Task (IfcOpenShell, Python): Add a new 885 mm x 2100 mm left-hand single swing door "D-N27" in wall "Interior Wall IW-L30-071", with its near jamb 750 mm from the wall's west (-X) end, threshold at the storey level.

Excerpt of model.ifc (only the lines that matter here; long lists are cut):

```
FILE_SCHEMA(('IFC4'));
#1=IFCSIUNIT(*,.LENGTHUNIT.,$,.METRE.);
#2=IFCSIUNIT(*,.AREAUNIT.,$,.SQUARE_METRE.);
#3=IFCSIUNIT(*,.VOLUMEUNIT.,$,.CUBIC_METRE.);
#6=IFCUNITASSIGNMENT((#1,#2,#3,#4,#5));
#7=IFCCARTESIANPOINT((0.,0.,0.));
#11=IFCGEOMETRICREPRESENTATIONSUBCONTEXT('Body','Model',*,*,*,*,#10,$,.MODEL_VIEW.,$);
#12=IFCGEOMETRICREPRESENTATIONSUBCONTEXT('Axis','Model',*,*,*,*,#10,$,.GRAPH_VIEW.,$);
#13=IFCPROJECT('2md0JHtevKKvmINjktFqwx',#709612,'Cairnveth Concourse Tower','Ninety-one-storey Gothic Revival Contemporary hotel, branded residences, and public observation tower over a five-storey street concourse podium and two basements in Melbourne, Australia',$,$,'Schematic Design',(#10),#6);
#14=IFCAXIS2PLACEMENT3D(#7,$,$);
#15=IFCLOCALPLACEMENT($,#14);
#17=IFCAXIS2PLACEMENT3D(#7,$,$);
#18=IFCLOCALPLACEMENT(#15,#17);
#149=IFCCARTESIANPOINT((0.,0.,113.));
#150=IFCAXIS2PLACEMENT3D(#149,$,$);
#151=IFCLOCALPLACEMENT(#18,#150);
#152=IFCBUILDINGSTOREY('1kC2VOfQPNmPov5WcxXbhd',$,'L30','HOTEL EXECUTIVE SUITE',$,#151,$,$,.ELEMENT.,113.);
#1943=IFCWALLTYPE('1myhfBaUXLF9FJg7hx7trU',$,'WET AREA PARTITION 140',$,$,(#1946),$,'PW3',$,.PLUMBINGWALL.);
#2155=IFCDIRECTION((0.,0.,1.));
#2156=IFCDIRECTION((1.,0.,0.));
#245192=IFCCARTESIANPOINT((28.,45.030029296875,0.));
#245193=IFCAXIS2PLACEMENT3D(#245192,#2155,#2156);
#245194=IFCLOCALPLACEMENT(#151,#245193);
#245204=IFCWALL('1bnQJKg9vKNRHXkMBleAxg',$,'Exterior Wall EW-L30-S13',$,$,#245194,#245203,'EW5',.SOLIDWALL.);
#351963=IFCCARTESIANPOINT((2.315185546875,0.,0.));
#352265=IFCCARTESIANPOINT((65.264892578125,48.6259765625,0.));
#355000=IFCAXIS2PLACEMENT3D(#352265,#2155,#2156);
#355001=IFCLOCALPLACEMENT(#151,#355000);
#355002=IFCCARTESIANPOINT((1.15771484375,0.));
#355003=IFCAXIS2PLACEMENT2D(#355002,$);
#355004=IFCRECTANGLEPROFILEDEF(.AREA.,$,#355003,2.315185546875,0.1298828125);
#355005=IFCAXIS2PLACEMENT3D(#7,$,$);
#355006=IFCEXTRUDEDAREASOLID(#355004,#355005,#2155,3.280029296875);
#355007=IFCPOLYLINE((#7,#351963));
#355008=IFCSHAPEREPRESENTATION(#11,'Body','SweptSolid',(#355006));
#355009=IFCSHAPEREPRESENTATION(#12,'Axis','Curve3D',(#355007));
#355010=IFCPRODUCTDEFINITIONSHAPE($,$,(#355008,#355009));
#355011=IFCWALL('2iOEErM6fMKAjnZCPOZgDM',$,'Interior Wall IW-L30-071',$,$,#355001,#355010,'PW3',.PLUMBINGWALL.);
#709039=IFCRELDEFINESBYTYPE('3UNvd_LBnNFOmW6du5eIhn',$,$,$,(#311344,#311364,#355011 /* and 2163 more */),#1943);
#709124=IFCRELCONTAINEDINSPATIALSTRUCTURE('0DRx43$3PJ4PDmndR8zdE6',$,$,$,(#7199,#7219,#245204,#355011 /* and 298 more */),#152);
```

```python
import numpy as np
import ifcopenshell
import ifcopenshell.api.feature
import ifcopenshell.api.geometry
import ifcopenshell.api.root
import ifcopenshell.api.spatial
import ifcopenshell.geom
import ifcopenshell.util.element
import ifcopenshell.util.placement
import ifcopenshell.util.representation
import ifcopenshell.util.shape
import ifcopenshell.util.unit

model = ifcopenshell.open("model.ifc")
unit_scale = ifcopenshell.util.unit.calculate_unit_scale(model)
settings = ifcopenshell.geom.settings()


def volume(element):
    """Net volume in cubic metres, openings subtracted."""
    shape = ifcopenshell.geom.create_shape(settings, element)
    return ifcopenshell.util.shape.get_volume(shape.geometry)


wall = model.by_guid("2iOEErM6fMKAjnZCPOZgDM")
storey = ifcopenshell.util.element.get_container(wall, ifc_class="IfcBuildingStorey")
context = ifcopenshell.util.representation.get_context(model, "Model", "Body", "MODEL_VIEW")
before = volume(wall)

width, height, from_end, sill = 0.885, 2.1, 0.75, 0.0  # metres

# The wall runs along its own X axis, and the end named is its -X end.
wall_shape = ifcopenshell.geom.create_shape(settings, wall)
x, y, z = ifcopenshell.util.shape.get_vertices(wall_shape.geometry).T
start = x.min() + from_end
face, thickness = float(y.min()), float(y.max() - y.min())
wall_matrix = ifcopenshell.util.placement.get_local_placement(wall.ObjectPlacement)
level = ifcopenshell.util.placement.get_local_placement(storey.ObjectPlacement)[2, 3]


def in_wall(x, y):
    """Placement at x, y metres in the wall's axes, at sill height."""
    matrix = wall_matrix.copy()
    matrix[:, 3] = wall_matrix @ np.array([x / unit_scale, y / unit_scale, 0.0, 1.0])
    matrix[2, 3] = level + sill / unit_scale
    return matrix


# Opening: a box that overshoots both wall faces by 50 mm.
opening = ifcopenshell.api.root.create_entity(model, ifc_class="IfcOpeningElement", predefined_type="OPENING")
box = ifcopenshell.api.geometry.add_wall_representation(
    model, context=context, length=width, height=height, thickness=thickness + 0.1
)
ifcopenshell.api.geometry.assign_representation(model, product=opening, representation=box)
ifcopenshell.api.geometry.edit_object_placement(model, product=opening, matrix=in_wall(start, face - 0.05), is_si=False)
ifcopenshell.api.feature.add_feature(model, feature=opening, element=wall)

door = ifcopenshell.api.root.create_entity(model, ifc_class="IfcDoor", name="D-N27", predefined_type="DOOR")
door.OverallWidth, door.OverallHeight = width / unit_scale, height / unit_scale
door.OperationType = "SINGLE_SWING_LEFT"
body = ifcopenshell.api.geometry.add_door_representation(
    model,
    context=context,
    overall_width=door.OverallWidth,
    overall_height=door.OverallHeight,
    operation_type="SINGLE_SWING_LEFT",
    lining_properties={"LiningDepth": thickness / unit_scale, "ThresholdDepth": thickness / unit_scale},
)
ifcopenshell.api.geometry.assign_representation(model, product=door, representation=body)
ifcopenshell.api.spatial.assign_container(model, products=[door], relating_structure=storey)
ifcopenshell.api.feature.add_filling(model, opening=opening, element=door)

# The lining spans the wall, so the door starts at the wall face.
ifcopenshell.api.geometry.edit_object_placement(model, product=door, matrix=in_wall(start, face), is_si=False)

after = volume(wall)

print(f"wall volume {before:.3f} -> {after:.3f} m3")

model.write("model-out.ifc")
```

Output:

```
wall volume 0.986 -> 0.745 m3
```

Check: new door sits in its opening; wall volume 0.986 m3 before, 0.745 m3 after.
